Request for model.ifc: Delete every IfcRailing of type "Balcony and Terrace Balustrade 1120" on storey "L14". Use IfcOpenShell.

First a look at what the model holds.

```python
import ifcopenshell
import ifcopenshell.util.element

model = ifcopenshell.open("model.ifc")
print(model.schema)
storey = next(s for s in model.by_type("IfcBuildingStorey") if s.Name == "L14")
railings = [e for e in ifcopenshell.util.element.get_decomposition(storey) if e.is_a("IfcRailing")]
seen = {}
for e in railings:
    element_type = ifcopenshell.util.element.get_type(e)
    name = element_type.Name if element_type not in (None, e) else None
    seen[name] = seen.get(name, 0) + 1
for name, count in sorted(seen.items(), key=str):
    print(count, "x", name)
```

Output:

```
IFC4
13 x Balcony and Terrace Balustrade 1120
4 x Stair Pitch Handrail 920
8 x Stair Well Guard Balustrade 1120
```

```python
import ifcopenshell
import ifcopenshell.api.root
import ifcopenshell.util.element

model = ifcopenshell.open("model.ifc")

storey = next(s for s in model.by_type("IfcBuildingStorey") if s.Name == "L14")
railings = [e for e in ifcopenshell.util.element.get_decomposition(storey) if e.is_a("IfcRailing")]
targets = [e for e in railings if (t := ifcopenshell.util.element.get_type(e)) not in (None, e) and t.Name == "Balcony and Terrace Balustrade 1120"]

for e in targets:
    ifcopenshell.api.root.remove_product(model, product=e)
print(len(targets), "removed")

model.write("model_edited.ifc")
```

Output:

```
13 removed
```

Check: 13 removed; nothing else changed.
